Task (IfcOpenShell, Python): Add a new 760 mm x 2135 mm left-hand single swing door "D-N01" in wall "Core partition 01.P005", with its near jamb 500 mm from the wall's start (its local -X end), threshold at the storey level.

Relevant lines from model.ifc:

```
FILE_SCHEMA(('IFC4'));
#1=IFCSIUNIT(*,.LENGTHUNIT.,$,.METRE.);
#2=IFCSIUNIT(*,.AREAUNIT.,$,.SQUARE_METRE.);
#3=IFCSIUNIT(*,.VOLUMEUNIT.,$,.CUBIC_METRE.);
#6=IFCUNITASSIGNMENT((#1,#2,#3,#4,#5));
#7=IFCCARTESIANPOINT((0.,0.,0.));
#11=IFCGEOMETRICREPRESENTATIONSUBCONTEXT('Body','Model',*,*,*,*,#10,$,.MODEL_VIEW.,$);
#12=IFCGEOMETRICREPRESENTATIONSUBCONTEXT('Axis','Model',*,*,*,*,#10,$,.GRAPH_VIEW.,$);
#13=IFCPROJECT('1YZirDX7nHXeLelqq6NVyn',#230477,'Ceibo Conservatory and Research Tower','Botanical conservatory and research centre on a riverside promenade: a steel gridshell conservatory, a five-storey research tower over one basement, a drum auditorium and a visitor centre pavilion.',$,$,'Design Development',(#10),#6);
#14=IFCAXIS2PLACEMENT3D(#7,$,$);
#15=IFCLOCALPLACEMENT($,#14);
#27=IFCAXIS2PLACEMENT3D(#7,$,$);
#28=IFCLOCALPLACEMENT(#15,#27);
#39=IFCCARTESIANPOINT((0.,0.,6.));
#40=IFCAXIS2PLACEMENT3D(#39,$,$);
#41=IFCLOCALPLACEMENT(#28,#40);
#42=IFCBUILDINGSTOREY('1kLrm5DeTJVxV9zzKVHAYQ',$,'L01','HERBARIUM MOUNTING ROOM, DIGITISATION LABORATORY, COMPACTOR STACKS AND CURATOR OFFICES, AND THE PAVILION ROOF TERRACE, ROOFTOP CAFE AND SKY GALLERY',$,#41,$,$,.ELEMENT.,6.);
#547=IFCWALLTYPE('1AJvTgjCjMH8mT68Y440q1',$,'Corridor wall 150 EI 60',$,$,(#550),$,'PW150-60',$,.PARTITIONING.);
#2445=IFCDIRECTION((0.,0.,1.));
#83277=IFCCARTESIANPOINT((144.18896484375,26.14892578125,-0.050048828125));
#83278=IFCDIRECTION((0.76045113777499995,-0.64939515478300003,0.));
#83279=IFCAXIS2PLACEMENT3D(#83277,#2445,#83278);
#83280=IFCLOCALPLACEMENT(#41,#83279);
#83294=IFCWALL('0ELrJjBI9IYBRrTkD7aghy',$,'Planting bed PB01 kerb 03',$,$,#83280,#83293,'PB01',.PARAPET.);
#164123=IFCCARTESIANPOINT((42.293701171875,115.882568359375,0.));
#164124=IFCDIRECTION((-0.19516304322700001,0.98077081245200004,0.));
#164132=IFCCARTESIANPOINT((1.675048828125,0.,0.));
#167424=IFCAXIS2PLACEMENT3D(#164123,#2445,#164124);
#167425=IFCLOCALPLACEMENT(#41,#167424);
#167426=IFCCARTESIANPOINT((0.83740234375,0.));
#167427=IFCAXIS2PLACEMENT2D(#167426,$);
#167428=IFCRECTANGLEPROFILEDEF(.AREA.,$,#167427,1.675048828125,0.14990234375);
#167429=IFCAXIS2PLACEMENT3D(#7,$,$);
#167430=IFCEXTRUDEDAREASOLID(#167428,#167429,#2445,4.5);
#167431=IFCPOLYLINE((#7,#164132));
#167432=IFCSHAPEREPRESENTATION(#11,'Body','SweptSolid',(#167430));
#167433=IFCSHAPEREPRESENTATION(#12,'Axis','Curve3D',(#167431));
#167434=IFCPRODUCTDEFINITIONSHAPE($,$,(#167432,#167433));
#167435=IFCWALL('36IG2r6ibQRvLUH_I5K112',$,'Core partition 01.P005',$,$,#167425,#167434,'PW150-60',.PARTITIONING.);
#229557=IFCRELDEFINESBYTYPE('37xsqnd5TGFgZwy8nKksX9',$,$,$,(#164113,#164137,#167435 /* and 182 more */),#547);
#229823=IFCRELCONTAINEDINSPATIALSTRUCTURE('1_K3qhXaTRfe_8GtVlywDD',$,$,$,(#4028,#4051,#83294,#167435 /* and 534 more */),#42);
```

```python
import numpy as np
import ifcopenshell
import ifcopenshell.api.feature
import ifcopenshell.api.geometry
import ifcopenshell.api.root
import ifcopenshell.api.spatial
import ifcopenshell.geom
import ifcopenshell.util.element
import ifcopenshell.util.placement
import ifcopenshell.util.representation
import ifcopenshell.util.shape
import ifcopenshell.util.unit

model = ifcopenshell.open("model.ifc")
unit_scale = ifcopenshell.util.unit.calculate_unit_scale(model)
settings = ifcopenshell.geom.settings()


def volume(element):
    """Net volume in cubic metres, openings subtracted."""
    shape = ifcopenshell.geom.create_shape(settings, element)
    return ifcopenshell.util.shape.get_volume(shape.geometry)


wall = model.by_id(167435)
storey = ifcopenshell.util.element.get_container(wall, ifc_class="IfcBuildingStorey")
context = ifcopenshell.util.representation.get_context(model, "Model", "Body", "MODEL_VIEW")
before = volume(wall)

width, height, from_end, sill = 0.76, 2.135, 0.5, 0.0  # metres

# The wall runs along its own X axis, and the end named is its -X end.
wall_shape = ifcopenshell.geom.create_shape(settings, wall)
x, y, z = ifcopenshell.util.shape.get_vertices(wall_shape.geometry).T
start = x.min() + from_end
face, thickness = float(y.min()), float(y.max() - y.min())
wall_matrix = ifcopenshell.util.placement.get_local_placement(wall.ObjectPlacement)
level = ifcopenshell.util.placement.get_local_placement(storey.ObjectPlacement)[2, 3]


def in_wall(x, y):
    """Placement at x, y metres in the wall's axes, at sill height."""
    matrix = wall_matrix.copy()
    matrix[:, 3] = wall_matrix @ np.array([x / unit_scale, y / unit_scale, 0.0, 1.0])
    matrix[2, 3] = level + sill / unit_scale
    return matrix


# Opening: a box that overshoots both wall faces by 50 mm.
opening = ifcopenshell.api.root.create_entity(model, ifc_class="IfcOpeningElement", predefined_type="OPENING")
box = ifcopenshell.api.geometry.add_wall_representation(
    model, context=context, length=width, height=height, thickness=thickness + 0.1
)
ifcopenshell.api.geometry.assign_representation(model, product=opening, representation=box)
ifcopenshell.api.geometry.edit_object_placement(model, product=opening, matrix=in_wall(start, face - 0.05), is_si=False)
ifcopenshell.api.feature.add_feature(model, feature=opening, element=wall)

door = ifcopenshell.api.root.create_entity(model, ifc_class="IfcDoor", name="D-N01", predefined_type="DOOR")
door.OverallWidth, door.OverallHeight = width / unit_scale, height / unit_scale
door.OperationType = "SINGLE_SWING_LEFT"
body = ifcopenshell.api.geometry.add_door_representation(
    model,
    context=context,
    overall_width=door.OverallWidth,
    overall_height=door.OverallHeight,
    operation_type="SINGLE_SWING_LEFT",
    lining_properties={"LiningDepth": thickness / unit_scale, "ThresholdDepth": thickness / unit_scale},
)
ifcopenshell.api.geometry.assign_representation(model, product=door, representation=body)
ifcopenshell.api.spatial.assign_container(model, products=[door], relating_structure=storey)
ifcopenshell.api.feature.add_filling(model, opening=opening, element=door)

# The lining spans the wall, so the door starts at the wall face.
ifcopenshell.api.geometry.edit_object_placement(model, product=door, matrix=in_wall(start, face), is_si=False)

after = volume(wall)

print(f"wall volume {before:.3f} -> {after:.3f} m3")

model.write("model_edited.ifc")
```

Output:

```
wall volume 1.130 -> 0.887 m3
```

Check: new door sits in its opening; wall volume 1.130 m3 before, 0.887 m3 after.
